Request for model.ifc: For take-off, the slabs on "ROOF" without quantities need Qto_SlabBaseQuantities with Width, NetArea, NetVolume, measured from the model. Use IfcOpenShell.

First a look at what the model holds.

```python
import ifcopenshell
import ifcopenshell.util.element
import ifcopenshell.util.unit

model = ifcopenshell.open("model.ifc")
print(model.schema)
for unit_type in ("LENGTHUNIT", "AREAUNIT", "VOLUMEUNIT"):
    print(unit_type, ifcopenshell.util.unit.calculate_unit_scale(model, unit_type))
storey = next(s for s in model.by_type("IfcBuildingStorey") if s.Name == "ROOF")
slabs = [e for e in ifcopenshell.util.element.get_decomposition(storey) if e.is_a("IfcSlab")]
for e in sorted(slabs, key=lambda e: e.id()):
    print(e.id(), e.is_a(), e.Name, list(ifcopenshell.util.element.get_psets(e, qtos_only=True)), sep=" | ")
```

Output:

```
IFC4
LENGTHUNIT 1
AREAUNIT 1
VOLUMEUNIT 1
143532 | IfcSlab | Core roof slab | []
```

```python
import ifcopenshell
import ifcopenshell.api.pset
import ifcopenshell.geom
import ifcopenshell.util.element
import ifcopenshell.util.shape
import ifcopenshell.util.unit

model = ifcopenshell.open("model.ifc")
unit_scale = ifcopenshell.util.unit.calculate_unit_scale(model)
area_scale = ifcopenshell.util.unit.calculate_unit_scale(model, "AREAUNIT")
volume_scale = ifcopenshell.util.unit.calculate_unit_scale(model, "VOLUMEUNIT")
settings = ifcopenshell.geom.settings()

storey = next(s for s in model.by_type("IfcBuildingStorey") if s.Name == "ROOF")
slabs = [e for e in ifcopenshell.util.element.get_decomposition(storey) if e.is_a("IfcSlab")]

for e in sorted(slabs, key=lambda e: e.id()):
    if ifcopenshell.util.element.get_psets(e, qtos_only=True, should_inherit=False):
        continue
    # Geometry comes back in metres, in the element's own axes.
    shape = ifcopenshell.geom.create_shape(settings, e)
    values = {
        "Width": ifcopenshell.util.shape.get_z(shape.geometry) / unit_scale,
        "NetArea": ifcopenshell.util.shape.get_footprint_area(shape.geometry) / area_scale,
        "NetVolume": ifcopenshell.util.shape.get_volume(shape.geometry) / volume_scale,
    }
    qto = ifcopenshell.api.pset.add_qto(model, product=e, name="Qto_SlabBaseQuantities")
    ifcopenshell.api.pset.edit_qto(model, qto=qto, properties=values)
    print(e.id(), {k: round(v, 3) for k, v in values.items()})

model.write("model-out.ifc")
```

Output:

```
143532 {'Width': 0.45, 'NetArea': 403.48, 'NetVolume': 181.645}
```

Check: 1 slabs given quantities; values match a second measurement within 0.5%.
